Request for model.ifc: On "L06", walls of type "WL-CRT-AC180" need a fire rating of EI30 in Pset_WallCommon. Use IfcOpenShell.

First a look at what the model holds.

```python
import ifcopenshell
import ifcopenshell.util.element

model = ifcopenshell.open("model.ifc")
print(model.schema)
storey = next(s for s in model.by_type("IfcBuildingStorey") if s.Name == "L06")
walls = [e for e in ifcopenshell.util.element.get_decomposition(storey) if e.is_a("IfcWall")]
seen = {}
for e in walls:
    element_type = ifcopenshell.util.element.get_type(e)
    key = (element_type.Name if element_type != e and element_type else None, ifcopenshell.util.element.get_pset(e, "Pset_WallCommon", "FireRating"))
    seen[key] = seen.get(key, 0) + 1
for (name, value), count in sorted(seen.items(), key=str):
    print(count, "x", name, "|", value)
```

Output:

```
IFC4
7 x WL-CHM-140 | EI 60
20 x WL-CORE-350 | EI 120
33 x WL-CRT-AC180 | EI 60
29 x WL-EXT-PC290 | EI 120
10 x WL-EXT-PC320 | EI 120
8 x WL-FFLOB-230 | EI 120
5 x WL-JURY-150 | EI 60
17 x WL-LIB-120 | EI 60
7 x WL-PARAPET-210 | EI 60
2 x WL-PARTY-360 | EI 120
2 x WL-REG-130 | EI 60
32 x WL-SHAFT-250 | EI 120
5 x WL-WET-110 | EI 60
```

```python
import ifcopenshell
import ifcopenshell.api.pset
import ifcopenshell.util.element

model = ifcopenshell.open("model.ifc")

storey = next(s for s in model.by_type("IfcBuildingStorey") if s.Name == "L06")
walls = [e for e in ifcopenshell.util.element.get_decomposition(storey) if e.is_a("IfcWall")]

count = 0
for e in walls:
    element_type = ifcopenshell.util.element.get_type(e)
    if element_type in (None, e) or element_type.Name != "WL-CRT-AC180":
        continue
    # add_pset returns the element's existing set when there is one.
    pset = ifcopenshell.api.pset.add_pset(model, product=e, name="Pset_WallCommon")
    ifcopenshell.api.pset.edit_pset(model, pset=pset, properties={"FireRating": "EI30"})
    count += 1

print(count, "walls updated")

model.write("model_rev.ifc")
```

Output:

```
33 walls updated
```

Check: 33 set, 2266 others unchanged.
